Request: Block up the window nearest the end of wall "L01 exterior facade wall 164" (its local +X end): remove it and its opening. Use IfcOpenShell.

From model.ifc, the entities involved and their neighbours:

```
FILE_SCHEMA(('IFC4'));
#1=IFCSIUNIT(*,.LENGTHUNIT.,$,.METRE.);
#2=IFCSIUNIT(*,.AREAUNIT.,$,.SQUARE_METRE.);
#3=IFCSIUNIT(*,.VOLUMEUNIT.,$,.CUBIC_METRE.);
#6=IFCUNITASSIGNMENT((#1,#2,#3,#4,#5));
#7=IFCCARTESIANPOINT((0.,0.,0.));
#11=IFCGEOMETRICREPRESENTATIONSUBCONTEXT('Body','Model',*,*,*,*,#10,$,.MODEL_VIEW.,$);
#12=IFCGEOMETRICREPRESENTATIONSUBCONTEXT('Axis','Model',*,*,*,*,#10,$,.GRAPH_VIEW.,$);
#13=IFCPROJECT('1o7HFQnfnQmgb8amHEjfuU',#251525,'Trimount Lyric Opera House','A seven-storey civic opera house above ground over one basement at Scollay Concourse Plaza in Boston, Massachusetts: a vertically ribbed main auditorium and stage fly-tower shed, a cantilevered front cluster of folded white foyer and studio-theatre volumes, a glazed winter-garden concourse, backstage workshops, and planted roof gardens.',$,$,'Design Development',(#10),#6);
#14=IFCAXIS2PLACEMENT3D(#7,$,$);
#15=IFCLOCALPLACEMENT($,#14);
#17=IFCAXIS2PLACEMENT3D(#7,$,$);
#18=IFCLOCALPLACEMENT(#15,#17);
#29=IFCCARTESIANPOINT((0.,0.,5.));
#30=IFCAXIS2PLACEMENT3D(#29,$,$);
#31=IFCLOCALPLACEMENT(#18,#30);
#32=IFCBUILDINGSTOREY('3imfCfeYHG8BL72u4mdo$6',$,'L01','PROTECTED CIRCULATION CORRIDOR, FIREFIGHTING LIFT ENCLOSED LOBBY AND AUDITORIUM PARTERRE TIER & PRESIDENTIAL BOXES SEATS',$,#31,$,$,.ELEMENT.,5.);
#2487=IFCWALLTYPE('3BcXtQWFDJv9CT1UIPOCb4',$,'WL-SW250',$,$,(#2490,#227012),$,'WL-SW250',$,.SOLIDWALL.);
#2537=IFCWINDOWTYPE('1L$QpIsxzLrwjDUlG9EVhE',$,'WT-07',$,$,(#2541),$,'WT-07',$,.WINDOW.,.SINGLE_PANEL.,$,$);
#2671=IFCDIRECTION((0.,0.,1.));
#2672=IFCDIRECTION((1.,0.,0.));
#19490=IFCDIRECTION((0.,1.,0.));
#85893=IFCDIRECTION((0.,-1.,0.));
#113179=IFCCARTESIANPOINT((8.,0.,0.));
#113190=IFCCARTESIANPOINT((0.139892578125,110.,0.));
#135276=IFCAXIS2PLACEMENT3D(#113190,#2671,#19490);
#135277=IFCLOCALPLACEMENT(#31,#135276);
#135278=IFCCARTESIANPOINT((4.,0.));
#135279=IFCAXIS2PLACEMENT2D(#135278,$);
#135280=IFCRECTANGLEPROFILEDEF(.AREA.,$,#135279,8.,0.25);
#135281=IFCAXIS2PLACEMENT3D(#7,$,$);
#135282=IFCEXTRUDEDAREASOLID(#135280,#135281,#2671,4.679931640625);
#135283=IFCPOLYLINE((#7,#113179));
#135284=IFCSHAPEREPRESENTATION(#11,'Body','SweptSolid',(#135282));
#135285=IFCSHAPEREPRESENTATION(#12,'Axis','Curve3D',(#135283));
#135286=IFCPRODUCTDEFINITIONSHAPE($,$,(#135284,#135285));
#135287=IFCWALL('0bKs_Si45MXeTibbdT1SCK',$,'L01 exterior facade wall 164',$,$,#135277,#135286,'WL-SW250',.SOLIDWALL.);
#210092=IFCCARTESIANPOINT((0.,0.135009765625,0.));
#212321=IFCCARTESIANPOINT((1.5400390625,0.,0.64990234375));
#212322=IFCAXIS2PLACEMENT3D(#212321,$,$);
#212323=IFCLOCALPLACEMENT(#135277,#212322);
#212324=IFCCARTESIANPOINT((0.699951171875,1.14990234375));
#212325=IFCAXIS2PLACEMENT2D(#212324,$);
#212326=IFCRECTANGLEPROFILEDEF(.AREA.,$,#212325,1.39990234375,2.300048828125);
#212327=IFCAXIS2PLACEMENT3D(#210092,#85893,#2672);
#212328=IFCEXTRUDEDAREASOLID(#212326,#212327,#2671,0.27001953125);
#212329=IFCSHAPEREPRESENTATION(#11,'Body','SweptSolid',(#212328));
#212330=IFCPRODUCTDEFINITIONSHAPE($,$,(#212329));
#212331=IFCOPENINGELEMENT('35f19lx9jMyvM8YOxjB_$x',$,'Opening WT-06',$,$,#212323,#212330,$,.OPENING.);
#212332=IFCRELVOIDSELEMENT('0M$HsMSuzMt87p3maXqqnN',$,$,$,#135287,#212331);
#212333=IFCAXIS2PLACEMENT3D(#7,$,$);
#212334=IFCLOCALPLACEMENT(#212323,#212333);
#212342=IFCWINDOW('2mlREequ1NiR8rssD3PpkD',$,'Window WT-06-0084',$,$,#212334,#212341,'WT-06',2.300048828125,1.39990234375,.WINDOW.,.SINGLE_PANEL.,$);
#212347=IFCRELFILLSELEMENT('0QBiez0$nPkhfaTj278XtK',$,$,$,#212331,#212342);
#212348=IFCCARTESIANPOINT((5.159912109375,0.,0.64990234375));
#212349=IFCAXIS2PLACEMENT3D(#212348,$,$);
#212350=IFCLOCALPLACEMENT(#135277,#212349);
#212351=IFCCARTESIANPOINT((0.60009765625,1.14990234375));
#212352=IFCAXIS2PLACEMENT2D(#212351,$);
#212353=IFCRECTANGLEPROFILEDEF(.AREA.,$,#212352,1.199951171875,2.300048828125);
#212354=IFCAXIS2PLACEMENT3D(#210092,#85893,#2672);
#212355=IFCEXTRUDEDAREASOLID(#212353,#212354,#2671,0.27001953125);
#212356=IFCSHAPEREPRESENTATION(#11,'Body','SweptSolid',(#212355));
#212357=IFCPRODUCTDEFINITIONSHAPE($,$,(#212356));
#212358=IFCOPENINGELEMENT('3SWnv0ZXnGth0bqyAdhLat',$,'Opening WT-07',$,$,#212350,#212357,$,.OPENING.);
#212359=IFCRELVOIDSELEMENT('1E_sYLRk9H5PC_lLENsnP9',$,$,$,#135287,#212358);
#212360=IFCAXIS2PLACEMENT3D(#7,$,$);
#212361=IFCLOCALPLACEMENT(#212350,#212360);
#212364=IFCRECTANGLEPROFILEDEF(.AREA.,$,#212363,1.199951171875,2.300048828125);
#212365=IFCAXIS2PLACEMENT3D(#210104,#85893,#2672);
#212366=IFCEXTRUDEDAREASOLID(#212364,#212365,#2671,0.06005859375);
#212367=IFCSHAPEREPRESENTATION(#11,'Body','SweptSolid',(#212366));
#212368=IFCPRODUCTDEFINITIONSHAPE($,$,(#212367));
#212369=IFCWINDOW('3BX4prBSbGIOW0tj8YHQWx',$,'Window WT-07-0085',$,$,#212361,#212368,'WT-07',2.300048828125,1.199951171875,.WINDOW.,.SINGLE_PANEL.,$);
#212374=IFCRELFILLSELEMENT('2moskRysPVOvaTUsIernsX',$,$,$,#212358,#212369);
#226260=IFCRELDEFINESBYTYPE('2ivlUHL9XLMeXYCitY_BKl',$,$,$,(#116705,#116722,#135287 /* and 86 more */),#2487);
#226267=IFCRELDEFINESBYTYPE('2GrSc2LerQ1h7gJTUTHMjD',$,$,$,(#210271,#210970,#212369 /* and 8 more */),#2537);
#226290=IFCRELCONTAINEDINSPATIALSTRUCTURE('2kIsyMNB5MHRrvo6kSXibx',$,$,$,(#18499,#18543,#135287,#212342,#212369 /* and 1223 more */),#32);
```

```python
import ifcopenshell
import ifcopenshell.api.feature
import ifcopenshell.api.root
import ifcopenshell.geom
import ifcopenshell.util.shape

model = ifcopenshell.open("model.ifc")
settings = ifcopenshell.geom.settings()


def volume(element):
    """Net volume in cubic metres, openings subtracted."""
    shape = ifcopenshell.geom.create_shape(settings, element)
    return ifcopenshell.util.shape.get_volume(shape.geometry)


window = model.by_id(212369)
opening = window.FillsVoids[0].RelatingOpeningElement
wall = opening.VoidsElements[0].RelatingBuildingElement
before = volume(wall)

ifcopenshell.api.root.remove_product(model, product=window)
ifcopenshell.api.feature.remove_feature(model, feature=opening)

after = volume(wall)

print(f"wall volume {before:.3f} -> {after:.3f} m3")

model.write("model-out.ifc")
```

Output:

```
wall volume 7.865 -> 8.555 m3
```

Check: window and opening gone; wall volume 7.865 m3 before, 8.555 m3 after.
